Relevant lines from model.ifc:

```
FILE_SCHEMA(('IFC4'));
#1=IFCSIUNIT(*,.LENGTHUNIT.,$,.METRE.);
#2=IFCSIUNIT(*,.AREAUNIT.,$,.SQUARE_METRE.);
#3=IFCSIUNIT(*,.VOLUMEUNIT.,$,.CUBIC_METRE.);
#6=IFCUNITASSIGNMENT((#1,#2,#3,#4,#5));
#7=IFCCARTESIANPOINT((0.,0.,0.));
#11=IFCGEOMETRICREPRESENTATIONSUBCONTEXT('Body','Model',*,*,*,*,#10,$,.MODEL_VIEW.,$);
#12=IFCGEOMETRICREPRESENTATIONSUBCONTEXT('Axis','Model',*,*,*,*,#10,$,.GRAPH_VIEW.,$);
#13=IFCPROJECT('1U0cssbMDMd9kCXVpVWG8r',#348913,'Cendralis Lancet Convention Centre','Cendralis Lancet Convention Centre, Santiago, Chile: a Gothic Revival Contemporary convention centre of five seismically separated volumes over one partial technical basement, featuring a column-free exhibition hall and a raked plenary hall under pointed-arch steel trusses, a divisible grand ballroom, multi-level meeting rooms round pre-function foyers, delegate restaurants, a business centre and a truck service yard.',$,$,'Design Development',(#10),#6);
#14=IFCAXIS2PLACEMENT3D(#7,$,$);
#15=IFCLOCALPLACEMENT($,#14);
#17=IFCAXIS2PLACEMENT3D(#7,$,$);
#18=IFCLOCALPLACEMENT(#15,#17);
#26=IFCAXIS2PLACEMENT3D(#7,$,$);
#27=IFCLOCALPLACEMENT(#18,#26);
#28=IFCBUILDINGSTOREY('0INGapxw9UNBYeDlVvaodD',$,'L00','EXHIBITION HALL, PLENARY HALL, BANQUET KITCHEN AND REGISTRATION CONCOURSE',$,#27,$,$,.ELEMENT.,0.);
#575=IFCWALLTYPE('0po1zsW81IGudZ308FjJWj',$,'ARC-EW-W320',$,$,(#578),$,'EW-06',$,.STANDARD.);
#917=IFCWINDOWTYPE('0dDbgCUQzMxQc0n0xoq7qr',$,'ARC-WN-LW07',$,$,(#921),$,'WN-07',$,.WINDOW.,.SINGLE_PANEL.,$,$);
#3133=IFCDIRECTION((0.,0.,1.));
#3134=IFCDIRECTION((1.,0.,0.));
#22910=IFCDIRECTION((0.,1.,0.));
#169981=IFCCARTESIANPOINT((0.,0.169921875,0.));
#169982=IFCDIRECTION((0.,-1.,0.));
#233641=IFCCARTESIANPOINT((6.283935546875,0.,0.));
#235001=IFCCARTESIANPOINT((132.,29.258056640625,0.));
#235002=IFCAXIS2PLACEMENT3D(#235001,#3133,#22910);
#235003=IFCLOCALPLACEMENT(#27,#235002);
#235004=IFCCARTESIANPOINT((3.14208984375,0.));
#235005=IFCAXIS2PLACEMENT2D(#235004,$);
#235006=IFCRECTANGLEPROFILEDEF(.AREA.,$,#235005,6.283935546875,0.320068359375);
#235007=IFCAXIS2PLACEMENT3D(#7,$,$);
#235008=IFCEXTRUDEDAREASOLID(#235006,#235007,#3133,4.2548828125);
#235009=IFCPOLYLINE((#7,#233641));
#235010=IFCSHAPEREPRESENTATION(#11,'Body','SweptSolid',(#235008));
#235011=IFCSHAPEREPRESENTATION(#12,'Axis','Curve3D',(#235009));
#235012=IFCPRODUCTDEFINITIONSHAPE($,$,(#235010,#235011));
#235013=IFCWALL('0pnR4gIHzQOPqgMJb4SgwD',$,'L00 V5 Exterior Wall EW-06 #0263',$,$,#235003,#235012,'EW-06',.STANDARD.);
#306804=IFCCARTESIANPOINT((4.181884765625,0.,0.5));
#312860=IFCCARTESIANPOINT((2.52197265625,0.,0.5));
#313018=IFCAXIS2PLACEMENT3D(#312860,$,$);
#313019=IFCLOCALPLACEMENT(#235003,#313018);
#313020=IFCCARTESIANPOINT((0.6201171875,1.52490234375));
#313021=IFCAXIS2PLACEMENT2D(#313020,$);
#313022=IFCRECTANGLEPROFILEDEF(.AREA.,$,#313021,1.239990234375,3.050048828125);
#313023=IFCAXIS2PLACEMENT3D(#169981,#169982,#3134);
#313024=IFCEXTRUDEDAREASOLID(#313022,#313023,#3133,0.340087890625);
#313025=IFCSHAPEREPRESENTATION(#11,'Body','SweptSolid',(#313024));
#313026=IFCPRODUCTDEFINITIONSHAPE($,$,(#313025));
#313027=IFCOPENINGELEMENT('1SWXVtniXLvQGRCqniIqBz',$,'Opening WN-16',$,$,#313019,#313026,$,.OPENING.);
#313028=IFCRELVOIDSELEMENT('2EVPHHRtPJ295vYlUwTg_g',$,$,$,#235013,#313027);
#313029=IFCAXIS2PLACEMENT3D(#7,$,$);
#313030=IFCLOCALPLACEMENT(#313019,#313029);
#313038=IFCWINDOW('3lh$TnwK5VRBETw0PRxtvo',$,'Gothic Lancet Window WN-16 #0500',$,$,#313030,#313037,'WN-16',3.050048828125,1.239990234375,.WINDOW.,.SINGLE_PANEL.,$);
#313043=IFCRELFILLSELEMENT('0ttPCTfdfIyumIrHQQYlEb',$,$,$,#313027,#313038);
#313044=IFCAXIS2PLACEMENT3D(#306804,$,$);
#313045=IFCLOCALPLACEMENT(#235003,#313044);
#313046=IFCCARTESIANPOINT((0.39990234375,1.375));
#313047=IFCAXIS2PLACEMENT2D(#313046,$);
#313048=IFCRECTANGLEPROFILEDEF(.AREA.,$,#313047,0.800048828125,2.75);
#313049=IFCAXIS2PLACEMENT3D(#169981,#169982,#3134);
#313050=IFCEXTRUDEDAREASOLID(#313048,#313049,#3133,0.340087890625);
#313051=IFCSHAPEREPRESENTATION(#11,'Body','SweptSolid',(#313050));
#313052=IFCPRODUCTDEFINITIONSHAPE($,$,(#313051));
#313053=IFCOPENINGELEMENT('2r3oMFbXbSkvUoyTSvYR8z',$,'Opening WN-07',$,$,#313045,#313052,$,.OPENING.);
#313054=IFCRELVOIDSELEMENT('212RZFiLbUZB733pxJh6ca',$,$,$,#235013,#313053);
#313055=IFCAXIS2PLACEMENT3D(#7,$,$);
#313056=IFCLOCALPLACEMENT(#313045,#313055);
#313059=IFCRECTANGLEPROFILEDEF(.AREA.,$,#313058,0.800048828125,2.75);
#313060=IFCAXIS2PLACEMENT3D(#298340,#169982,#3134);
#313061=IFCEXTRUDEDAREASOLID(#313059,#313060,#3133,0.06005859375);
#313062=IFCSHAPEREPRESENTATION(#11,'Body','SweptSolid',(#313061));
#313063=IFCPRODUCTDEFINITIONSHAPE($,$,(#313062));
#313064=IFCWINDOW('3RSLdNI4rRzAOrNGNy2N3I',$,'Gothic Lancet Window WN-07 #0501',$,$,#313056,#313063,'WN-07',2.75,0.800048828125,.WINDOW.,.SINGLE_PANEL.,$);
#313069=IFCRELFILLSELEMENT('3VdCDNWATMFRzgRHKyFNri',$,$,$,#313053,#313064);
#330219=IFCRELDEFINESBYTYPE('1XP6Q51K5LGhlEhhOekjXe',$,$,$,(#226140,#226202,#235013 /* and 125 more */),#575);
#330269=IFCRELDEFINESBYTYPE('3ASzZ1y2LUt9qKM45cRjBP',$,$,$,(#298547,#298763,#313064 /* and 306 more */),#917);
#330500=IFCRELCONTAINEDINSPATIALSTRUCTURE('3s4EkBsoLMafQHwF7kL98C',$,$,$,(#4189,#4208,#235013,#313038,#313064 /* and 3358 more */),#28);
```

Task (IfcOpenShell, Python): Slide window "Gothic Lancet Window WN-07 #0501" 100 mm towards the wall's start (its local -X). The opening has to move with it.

```python
import ifcopenshell
import ifcopenshell.api.geometry
import ifcopenshell.util.placement

model = ifcopenshell.open("model.ifc")

window = model.by_guid("3RSLdNI4rRzAOrNGNy2N3I")
opening = window.FillsVoids[0].RelatingOpeningElement
wall = opening.VoidsElements[0].RelatingBuildingElement

wall_matrix = ifcopenshell.util.placement.get_local_placement(wall.ObjectPlacement)
shift = wall_matrix[:3, 0] * -0.1
before = ifcopenshell.util.placement.get_local_placement(window.ObjectPlacement)[:3, 3].copy()

# The window is placed relative to its opening, so it follows when the opening moves.
matrix = ifcopenshell.util.placement.get_local_placement(opening.ObjectPlacement)
matrix[:3, 3] += shift
ifcopenshell.api.geometry.edit_object_placement(
    model, product=opening, matrix=matrix, is_si=False, should_transform_children=True
)

after = ifcopenshell.util.placement.get_local_placement(window.ObjectPlacement)[:3, 3]
print("window moved by", (after - before).round(3) + 0.0)

model.write("model_v2.ifc")
```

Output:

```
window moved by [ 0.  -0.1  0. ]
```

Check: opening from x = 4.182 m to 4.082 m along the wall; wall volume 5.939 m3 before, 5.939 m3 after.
